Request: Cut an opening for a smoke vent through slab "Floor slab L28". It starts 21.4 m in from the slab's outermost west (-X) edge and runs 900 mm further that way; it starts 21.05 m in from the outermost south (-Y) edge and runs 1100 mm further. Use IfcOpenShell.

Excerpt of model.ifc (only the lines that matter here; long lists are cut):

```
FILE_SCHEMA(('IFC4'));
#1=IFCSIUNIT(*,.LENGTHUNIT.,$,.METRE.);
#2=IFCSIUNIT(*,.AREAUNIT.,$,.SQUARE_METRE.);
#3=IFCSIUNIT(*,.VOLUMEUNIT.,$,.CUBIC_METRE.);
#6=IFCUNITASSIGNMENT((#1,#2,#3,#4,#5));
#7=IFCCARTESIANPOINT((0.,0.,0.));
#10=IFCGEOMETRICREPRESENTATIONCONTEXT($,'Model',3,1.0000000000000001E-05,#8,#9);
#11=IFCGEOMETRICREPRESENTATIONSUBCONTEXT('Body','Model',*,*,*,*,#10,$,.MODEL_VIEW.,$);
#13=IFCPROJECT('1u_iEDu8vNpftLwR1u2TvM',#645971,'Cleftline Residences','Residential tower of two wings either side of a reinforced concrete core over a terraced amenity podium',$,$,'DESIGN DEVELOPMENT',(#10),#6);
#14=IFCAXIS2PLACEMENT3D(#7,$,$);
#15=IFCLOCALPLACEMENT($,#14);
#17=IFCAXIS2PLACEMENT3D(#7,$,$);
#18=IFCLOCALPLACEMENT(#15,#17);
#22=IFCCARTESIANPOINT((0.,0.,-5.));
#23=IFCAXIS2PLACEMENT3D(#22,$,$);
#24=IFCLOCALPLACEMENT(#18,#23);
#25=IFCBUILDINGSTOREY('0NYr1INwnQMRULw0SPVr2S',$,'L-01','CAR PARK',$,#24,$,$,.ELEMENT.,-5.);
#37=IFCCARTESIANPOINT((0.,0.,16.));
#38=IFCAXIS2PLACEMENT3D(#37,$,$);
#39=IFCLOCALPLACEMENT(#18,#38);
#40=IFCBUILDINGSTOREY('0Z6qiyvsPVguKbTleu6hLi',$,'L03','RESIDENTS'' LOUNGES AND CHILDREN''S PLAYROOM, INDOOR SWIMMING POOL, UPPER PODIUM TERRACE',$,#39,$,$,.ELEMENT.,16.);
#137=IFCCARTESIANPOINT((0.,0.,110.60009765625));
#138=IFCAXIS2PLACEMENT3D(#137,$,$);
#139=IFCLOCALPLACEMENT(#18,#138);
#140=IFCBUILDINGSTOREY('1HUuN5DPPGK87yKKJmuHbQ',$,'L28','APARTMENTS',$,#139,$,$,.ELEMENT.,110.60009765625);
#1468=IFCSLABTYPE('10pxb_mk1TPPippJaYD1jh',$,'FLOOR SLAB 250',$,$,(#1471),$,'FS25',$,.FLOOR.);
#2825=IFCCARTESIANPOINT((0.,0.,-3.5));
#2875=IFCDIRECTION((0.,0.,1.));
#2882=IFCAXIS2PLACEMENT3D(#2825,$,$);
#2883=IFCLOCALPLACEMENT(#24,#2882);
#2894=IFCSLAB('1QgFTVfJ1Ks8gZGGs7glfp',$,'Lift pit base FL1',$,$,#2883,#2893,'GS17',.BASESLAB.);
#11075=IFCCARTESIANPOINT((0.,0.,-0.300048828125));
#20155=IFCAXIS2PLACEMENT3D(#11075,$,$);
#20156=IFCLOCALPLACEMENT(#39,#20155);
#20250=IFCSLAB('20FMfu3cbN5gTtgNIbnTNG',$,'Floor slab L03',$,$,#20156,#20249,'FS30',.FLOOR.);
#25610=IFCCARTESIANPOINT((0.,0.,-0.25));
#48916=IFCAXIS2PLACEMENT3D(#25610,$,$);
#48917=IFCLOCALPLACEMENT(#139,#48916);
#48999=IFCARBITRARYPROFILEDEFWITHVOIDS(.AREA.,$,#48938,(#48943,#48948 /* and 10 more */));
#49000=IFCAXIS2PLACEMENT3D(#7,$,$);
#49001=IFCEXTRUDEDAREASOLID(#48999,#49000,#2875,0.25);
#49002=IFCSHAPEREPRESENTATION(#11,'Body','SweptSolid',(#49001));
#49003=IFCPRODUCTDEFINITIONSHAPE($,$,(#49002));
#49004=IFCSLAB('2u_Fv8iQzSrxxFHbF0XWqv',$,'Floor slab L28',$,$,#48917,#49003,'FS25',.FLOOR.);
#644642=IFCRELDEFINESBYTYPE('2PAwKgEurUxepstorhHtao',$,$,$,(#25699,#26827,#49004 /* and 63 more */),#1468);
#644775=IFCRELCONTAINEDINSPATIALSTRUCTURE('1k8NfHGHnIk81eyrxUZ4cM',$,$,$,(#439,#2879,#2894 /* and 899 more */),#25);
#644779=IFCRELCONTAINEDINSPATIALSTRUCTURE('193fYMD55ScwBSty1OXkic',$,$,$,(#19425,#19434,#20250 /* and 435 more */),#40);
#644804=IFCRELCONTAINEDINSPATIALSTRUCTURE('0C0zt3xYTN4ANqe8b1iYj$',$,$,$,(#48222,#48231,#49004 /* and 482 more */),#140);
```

```python
import numpy as np
import ifcopenshell
import ifcopenshell.api.feature
import ifcopenshell.api.geometry
import ifcopenshell.api.root
import ifcopenshell.geom
import ifcopenshell.util.placement
import ifcopenshell.util.representation
import ifcopenshell.util.shape
import ifcopenshell.util.unit

model = ifcopenshell.open("model.ifc")
unit_scale = ifcopenshell.util.unit.calculate_unit_scale(model)
settings = ifcopenshell.geom.settings()


def volume(element):
    """Net volume in cubic metres, openings subtracted."""
    shape = ifcopenshell.geom.create_shape(settings, element)
    return ifcopenshell.util.shape.get_volume(shape.geometry)


slab = model.by_guid("2u_Fv8iQzSrxxFHbF0XWqv")
before = volume(slab)

# Extent in the slab's own axes, in metres. The edges named are its -X and -Y sides.
slab_shape = ifcopenshell.geom.create_shape(settings, slab)
vertices = ifcopenshell.util.shape.get_vertices(slab_shape.geometry)
x_min, y_min, bottom = vertices.min(axis=0)
top = vertices[:, 2].max()

opening = ifcopenshell.api.root.create_entity(model, ifc_class="IfcOpeningElement", name="Smoke vent opening", predefined_type="OPENING")
context = ifcopenshell.util.representation.get_context(model, "Model", "Body", "MODEL_VIEW")
width, depth = 0.9, 1.1
outline = [(0.0, 0.0), (width, 0.0), (width, depth), (0.0, depth), (0.0, 0.0)]
# Overshoot both faces by 50 mm so the cut is clean.
shape = ifcopenshell.api.geometry.add_slab_representation(
    model, context=context, depth=top - bottom + 0.1, polyline=outline
)
ifcopenshell.api.geometry.assign_representation(model, product=opening, representation=shape)

matrix = ifcopenshell.util.placement.get_local_placement(slab.ObjectPlacement)
matrix[:, 3] = matrix @ np.append(np.array([x_min + 21.4, y_min + 21.05, bottom - 0.05]) / unit_scale, 1.0)
ifcopenshell.api.geometry.edit_object_placement(model, product=opening, matrix=matrix, is_si=False)
ifcopenshell.api.feature.add_feature(model, feature=opening, element=slab)

after = volume(slab)

print(f"slab volume {before:.3f} -> {after:.3f} m3")

model.write("model_rev.ifc")
```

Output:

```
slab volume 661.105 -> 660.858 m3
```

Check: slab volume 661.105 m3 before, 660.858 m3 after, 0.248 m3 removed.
